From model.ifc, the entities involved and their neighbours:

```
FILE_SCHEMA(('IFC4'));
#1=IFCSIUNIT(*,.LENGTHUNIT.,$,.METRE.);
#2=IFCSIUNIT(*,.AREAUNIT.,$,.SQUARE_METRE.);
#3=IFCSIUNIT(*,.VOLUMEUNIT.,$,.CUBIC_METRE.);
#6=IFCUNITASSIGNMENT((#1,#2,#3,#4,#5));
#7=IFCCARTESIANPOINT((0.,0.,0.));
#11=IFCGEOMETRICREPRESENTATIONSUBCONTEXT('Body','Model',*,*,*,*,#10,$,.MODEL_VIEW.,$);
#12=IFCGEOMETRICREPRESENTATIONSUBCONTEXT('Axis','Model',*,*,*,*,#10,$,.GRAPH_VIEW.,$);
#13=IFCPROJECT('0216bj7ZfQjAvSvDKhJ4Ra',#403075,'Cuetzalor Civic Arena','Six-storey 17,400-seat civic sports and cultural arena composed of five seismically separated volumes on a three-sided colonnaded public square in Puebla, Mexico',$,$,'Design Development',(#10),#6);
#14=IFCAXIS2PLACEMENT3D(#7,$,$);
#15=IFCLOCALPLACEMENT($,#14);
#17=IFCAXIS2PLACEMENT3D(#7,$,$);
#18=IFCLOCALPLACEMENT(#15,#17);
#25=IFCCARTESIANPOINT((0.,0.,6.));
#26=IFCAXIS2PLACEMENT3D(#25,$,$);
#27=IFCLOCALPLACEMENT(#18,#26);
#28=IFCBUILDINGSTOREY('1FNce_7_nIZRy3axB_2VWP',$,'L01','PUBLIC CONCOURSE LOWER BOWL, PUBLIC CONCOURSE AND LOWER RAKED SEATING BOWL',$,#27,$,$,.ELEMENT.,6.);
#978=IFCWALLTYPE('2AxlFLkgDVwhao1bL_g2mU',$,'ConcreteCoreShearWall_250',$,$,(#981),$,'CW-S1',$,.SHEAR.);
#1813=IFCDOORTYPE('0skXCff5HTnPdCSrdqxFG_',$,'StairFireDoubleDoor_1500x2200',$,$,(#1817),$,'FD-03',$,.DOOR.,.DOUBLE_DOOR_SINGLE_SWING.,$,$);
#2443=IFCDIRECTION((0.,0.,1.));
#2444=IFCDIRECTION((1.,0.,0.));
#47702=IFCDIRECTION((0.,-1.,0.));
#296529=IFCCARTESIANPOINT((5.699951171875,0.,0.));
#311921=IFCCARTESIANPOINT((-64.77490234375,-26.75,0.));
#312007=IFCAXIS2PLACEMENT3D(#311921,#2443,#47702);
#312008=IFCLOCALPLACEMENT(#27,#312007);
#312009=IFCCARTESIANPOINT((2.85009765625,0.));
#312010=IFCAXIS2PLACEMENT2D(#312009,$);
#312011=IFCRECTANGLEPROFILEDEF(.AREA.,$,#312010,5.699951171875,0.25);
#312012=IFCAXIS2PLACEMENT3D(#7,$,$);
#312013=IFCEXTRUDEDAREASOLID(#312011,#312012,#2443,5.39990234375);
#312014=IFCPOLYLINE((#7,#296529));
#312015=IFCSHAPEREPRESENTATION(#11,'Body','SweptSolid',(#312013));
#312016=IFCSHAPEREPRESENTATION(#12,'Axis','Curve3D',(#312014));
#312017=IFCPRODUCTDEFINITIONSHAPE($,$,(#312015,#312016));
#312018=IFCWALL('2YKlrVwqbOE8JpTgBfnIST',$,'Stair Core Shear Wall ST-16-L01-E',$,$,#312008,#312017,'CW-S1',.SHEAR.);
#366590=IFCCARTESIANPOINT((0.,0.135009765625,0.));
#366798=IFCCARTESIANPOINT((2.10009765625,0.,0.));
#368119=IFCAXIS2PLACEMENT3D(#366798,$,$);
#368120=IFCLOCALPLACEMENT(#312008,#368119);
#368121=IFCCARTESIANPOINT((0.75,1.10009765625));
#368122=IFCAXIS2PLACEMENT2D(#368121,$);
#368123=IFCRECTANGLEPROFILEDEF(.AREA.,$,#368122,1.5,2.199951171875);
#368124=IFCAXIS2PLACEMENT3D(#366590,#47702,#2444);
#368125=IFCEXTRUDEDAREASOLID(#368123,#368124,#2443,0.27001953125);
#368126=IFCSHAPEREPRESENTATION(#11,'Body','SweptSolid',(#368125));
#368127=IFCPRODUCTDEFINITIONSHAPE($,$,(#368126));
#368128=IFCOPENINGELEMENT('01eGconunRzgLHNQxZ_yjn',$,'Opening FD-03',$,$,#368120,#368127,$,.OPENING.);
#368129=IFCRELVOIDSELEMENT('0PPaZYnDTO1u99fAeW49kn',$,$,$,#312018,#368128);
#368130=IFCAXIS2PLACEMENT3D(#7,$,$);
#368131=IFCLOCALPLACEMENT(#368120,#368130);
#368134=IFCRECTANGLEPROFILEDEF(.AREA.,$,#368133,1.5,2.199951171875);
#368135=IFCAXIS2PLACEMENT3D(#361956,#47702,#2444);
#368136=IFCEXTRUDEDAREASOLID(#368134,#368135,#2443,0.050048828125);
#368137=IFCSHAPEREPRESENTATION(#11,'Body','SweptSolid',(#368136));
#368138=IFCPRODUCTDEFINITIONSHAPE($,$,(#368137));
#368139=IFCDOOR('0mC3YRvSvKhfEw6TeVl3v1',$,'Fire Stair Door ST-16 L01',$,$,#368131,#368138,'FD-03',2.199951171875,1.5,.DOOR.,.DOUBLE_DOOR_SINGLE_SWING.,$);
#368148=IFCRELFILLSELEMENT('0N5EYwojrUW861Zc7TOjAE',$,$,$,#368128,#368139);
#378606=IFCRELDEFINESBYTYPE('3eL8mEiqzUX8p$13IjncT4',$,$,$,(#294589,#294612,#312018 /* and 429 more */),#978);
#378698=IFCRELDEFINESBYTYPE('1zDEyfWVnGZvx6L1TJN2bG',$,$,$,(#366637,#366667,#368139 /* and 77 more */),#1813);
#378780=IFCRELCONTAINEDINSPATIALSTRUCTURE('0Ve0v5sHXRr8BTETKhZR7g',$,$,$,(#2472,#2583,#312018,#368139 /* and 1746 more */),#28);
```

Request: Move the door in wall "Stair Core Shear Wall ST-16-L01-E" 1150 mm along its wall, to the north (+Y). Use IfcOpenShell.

```python
import ifcopenshell
import ifcopenshell.api.geometry
import ifcopenshell.util.placement

model = ifcopenshell.open("model.ifc")

door = model.by_guid("0mC3YRvSvKhfEw6TeVl3v1")
opening = door.FillsVoids[0].RelatingOpeningElement
wall = opening.VoidsElements[0].RelatingBuildingElement

wall_matrix = ifcopenshell.util.placement.get_local_placement(wall.ObjectPlacement)
shift = wall_matrix[:3, 0] * -1.15
before = ifcopenshell.util.placement.get_local_placement(door.ObjectPlacement)[:3, 3].copy()

# The door is placed relative to its opening, so it follows when the opening moves.
matrix = ifcopenshell.util.placement.get_local_placement(opening.ObjectPlacement)
matrix[:3, 3] += shift
ifcopenshell.api.geometry.edit_object_placement(
    model, product=opening, matrix=matrix, is_si=False, should_transform_children=True
)

after = ifcopenshell.util.placement.get_local_placement(door.ObjectPlacement)[:3, 3]
print("door moved by", (after - before).round(3) + 0.0)

model.write("model_rev.ifc")
```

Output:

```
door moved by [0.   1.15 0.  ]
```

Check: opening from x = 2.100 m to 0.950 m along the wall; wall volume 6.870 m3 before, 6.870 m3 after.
